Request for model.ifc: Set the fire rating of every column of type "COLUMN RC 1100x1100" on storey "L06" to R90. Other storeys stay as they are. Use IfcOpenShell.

First a look at what the model holds.

```python
import ifcopenshell
import ifcopenshell.util.element

model = ifcopenshell.open("model.ifc")
print(model.schema)
storey = next(s for s in model.by_type("IfcBuildingStorey") if s.Name == "L06")
columns = [e for e in ifcopenshell.util.element.get_decomposition(storey) if e.is_a("IfcColumn")]
seen = {}
for e in columns:
    element_type = ifcopenshell.util.element.get_type(e)
    key = (element_type.Name if element_type != e and element_type else None, ifcopenshell.util.element.get_pset(e, "Pset_ColumnCommon", "FireRating"))
    seen[key] = seen.get(key, 0) + 1
for (name, value), count in sorted(seen.items(), key=str):
    print(count, "x", name, "|", value)
```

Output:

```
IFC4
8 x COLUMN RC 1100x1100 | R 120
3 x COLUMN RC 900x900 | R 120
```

```python
import ifcopenshell
import ifcopenshell.api.pset
import ifcopenshell.util.element

model = ifcopenshell.open("model.ifc")

storey = next(s for s in model.by_type("IfcBuildingStorey") if s.Name == "L06")
columns = [e for e in ifcopenshell.util.element.get_decomposition(storey) if e.is_a("IfcColumn")]

count = 0
for e in columns:
    element_type = ifcopenshell.util.element.get_type(e)
    if element_type in (None, e) or element_type.Name != "COLUMN RC 1100x1100":
        continue
    found = ifcopenshell.util.element.get_pset(e, "Pset_ColumnCommon", should_inherit=False)
    if found:
        pset = model.by_id(found["id"])
        if len(ifcopenshell.util.element.get_elements_by_pset(pset)) > 1:
            pset = ifcopenshell.api.pset.unshare_pset(model, products=[e], pset=pset)[0]
    else:
        pset = ifcopenshell.api.pset.add_pset(model, product=e, name="Pset_ColumnCommon")
    ifcopenshell.api.pset.edit_pset(model, pset=pset, properties={"FireRating": "R90"})
    count += 1

print(count, "columns updated")

model.write("model_updated.ifc")
```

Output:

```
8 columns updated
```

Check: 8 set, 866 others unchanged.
